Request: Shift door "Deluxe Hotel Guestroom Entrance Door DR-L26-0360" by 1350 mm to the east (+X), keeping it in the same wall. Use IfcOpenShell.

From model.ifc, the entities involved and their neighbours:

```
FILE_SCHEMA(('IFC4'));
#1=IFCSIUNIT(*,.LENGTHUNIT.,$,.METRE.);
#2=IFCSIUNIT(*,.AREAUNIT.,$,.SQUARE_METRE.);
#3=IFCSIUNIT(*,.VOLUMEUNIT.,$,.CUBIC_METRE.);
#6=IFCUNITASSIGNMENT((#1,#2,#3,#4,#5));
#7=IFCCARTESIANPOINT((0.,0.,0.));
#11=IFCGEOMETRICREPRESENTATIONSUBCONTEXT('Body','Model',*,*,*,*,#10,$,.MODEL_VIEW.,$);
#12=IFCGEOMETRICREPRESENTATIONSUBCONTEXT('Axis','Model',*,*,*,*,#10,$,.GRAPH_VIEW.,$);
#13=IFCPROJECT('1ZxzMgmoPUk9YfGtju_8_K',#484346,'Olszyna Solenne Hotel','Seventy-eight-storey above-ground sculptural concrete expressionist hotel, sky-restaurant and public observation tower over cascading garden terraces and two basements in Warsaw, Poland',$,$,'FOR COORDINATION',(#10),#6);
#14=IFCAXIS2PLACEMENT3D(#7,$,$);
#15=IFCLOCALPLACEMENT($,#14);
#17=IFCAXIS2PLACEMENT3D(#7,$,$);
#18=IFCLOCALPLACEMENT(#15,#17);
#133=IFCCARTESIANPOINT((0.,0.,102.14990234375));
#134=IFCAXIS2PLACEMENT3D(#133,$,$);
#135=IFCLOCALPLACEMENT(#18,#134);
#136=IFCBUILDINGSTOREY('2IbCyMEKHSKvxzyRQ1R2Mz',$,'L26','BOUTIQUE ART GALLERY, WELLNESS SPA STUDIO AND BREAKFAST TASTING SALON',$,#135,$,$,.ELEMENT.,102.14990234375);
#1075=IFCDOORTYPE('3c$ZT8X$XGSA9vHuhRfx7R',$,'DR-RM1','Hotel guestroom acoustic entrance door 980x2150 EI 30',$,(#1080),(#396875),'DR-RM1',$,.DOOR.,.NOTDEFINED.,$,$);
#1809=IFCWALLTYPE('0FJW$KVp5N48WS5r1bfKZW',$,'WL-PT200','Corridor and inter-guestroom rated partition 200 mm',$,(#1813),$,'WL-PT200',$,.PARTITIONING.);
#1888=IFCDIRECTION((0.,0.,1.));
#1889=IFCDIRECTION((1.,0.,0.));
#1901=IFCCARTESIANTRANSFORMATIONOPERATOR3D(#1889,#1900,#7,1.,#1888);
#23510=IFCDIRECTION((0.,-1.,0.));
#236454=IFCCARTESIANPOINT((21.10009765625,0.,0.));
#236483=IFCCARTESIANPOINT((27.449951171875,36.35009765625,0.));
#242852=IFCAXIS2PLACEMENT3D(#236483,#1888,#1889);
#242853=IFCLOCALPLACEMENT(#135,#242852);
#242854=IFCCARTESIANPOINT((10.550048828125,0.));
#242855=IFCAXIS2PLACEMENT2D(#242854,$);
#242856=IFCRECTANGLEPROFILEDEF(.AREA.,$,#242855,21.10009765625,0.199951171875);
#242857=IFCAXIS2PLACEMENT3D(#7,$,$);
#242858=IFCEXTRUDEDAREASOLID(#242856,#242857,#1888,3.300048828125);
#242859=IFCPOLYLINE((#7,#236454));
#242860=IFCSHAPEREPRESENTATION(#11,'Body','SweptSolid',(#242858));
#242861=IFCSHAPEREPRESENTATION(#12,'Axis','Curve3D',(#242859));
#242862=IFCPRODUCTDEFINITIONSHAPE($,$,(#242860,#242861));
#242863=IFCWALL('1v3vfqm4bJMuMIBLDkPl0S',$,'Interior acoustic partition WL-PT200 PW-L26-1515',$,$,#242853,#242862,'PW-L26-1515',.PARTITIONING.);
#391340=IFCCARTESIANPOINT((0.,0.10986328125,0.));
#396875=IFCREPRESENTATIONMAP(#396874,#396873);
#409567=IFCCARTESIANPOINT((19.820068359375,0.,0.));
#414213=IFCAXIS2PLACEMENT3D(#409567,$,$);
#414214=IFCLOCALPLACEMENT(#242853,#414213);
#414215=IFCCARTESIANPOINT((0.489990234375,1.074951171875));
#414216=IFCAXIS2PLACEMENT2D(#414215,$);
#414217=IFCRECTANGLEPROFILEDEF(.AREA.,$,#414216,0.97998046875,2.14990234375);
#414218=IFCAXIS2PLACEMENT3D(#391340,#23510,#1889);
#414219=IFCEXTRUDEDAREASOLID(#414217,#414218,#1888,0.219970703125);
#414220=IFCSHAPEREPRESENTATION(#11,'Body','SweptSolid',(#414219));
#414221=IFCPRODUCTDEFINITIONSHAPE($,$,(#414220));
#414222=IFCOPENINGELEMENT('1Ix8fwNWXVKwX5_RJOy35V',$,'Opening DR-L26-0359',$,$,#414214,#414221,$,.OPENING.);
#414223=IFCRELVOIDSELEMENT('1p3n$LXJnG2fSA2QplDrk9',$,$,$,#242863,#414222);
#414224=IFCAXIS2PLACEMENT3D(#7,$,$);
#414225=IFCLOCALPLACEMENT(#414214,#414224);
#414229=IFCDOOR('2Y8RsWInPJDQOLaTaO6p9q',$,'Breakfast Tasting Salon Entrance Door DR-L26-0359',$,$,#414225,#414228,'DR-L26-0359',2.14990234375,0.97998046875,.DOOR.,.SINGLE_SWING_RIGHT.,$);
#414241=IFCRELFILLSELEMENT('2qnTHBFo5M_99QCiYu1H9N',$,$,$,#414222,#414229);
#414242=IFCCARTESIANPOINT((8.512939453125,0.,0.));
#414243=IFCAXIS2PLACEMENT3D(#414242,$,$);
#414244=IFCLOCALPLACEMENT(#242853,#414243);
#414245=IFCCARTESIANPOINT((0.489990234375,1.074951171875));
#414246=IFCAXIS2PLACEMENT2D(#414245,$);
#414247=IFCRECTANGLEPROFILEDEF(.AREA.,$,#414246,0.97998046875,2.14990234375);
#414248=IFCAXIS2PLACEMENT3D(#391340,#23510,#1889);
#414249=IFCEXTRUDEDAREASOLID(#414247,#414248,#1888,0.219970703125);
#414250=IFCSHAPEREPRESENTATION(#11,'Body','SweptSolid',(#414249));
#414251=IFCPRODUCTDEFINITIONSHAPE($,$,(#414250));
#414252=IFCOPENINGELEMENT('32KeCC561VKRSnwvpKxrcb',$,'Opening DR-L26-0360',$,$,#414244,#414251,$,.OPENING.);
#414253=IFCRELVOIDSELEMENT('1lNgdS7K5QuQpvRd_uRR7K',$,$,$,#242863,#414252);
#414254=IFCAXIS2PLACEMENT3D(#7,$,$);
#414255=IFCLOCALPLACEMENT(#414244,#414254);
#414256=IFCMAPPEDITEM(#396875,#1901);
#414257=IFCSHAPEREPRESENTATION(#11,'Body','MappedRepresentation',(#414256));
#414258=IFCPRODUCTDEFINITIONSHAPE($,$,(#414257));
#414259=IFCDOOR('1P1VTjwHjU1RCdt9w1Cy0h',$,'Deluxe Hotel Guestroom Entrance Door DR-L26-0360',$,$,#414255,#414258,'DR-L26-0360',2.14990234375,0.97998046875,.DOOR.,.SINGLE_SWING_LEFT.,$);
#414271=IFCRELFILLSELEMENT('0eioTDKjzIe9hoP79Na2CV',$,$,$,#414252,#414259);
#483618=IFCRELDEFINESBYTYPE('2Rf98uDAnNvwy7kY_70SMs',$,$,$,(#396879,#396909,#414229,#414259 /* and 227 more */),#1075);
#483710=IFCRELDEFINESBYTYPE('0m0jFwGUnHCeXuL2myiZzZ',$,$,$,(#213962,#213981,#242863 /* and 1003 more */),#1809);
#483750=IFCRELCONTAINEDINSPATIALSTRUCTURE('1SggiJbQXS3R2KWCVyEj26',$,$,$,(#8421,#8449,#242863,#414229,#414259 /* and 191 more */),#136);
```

```python
import ifcopenshell
import ifcopenshell.api.geometry
import ifcopenshell.util.placement

model = ifcopenshell.open("model.ifc")

door = model.by_guid("1P1VTjwHjU1RCdt9w1Cy0h")
opening = door.FillsVoids[0].RelatingOpeningElement
wall = opening.VoidsElements[0].RelatingBuildingElement

wall_matrix = ifcopenshell.util.placement.get_local_placement(wall.ObjectPlacement)
shift = wall_matrix[:3, 0] * 1.35
before = ifcopenshell.util.placement.get_local_placement(door.ObjectPlacement)[:3, 3].copy()

# The door is placed relative to its opening, so it follows when the opening moves.
matrix = ifcopenshell.util.placement.get_local_placement(opening.ObjectPlacement)
matrix[:3, 3] += shift
ifcopenshell.api.geometry.edit_object_placement(
    model, product=opening, matrix=matrix, is_si=False, should_transform_children=True
)

after = ifcopenshell.util.placement.get_local_placement(door.ObjectPlacement)[:3, 3]
print("door moved by", (after - before).round(3) + 0.0)

model.write("model_v2.ifc")
```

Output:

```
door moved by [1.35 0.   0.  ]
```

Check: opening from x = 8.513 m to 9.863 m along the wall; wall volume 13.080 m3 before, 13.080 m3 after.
